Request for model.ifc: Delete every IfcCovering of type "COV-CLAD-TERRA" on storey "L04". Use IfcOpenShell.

First a look at what the model holds.

```python
import ifcopenshell
import ifcopenshell.util.element

model = ifcopenshell.open("model.ifc")
print(model.schema)
storey = next(s for s in model.by_type("IfcBuildingStorey") if s.Name == "L04")
coverings = [e for e in ifcopenshell.util.element.get_decomposition(storey) if e.is_a("IfcCovering")]
seen = {}
for e in coverings:
    element_type = ifcopenshell.util.element.get_type(e)
    name = element_type.Name if element_type not in (None, e) else None
    seen[name] = seen.get(name, 0) + 1
for name, count in sorted(seen.items(), key=str):
    print(count, "x", name)
```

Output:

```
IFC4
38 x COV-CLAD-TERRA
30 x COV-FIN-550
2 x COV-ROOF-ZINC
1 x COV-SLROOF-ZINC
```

```python
import ifcopenshell
import ifcopenshell.api.root
import ifcopenshell.util.element

model = ifcopenshell.open("model.ifc")

storey = next(s for s in model.by_type("IfcBuildingStorey") if s.Name == "L04")
coverings = [e for e in ifcopenshell.util.element.get_decomposition(storey) if e.is_a("IfcCovering")]
targets = [e for e in coverings if (t := ifcopenshell.util.element.get_type(e)) not in (None, e) and t.Name == "COV-CLAD-TERRA"]

for e in targets:
    ifcopenshell.api.root.remove_product(model, product=e)
print(len(targets), "removed")

model.write("model_edited.ifc")
```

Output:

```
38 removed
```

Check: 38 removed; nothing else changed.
